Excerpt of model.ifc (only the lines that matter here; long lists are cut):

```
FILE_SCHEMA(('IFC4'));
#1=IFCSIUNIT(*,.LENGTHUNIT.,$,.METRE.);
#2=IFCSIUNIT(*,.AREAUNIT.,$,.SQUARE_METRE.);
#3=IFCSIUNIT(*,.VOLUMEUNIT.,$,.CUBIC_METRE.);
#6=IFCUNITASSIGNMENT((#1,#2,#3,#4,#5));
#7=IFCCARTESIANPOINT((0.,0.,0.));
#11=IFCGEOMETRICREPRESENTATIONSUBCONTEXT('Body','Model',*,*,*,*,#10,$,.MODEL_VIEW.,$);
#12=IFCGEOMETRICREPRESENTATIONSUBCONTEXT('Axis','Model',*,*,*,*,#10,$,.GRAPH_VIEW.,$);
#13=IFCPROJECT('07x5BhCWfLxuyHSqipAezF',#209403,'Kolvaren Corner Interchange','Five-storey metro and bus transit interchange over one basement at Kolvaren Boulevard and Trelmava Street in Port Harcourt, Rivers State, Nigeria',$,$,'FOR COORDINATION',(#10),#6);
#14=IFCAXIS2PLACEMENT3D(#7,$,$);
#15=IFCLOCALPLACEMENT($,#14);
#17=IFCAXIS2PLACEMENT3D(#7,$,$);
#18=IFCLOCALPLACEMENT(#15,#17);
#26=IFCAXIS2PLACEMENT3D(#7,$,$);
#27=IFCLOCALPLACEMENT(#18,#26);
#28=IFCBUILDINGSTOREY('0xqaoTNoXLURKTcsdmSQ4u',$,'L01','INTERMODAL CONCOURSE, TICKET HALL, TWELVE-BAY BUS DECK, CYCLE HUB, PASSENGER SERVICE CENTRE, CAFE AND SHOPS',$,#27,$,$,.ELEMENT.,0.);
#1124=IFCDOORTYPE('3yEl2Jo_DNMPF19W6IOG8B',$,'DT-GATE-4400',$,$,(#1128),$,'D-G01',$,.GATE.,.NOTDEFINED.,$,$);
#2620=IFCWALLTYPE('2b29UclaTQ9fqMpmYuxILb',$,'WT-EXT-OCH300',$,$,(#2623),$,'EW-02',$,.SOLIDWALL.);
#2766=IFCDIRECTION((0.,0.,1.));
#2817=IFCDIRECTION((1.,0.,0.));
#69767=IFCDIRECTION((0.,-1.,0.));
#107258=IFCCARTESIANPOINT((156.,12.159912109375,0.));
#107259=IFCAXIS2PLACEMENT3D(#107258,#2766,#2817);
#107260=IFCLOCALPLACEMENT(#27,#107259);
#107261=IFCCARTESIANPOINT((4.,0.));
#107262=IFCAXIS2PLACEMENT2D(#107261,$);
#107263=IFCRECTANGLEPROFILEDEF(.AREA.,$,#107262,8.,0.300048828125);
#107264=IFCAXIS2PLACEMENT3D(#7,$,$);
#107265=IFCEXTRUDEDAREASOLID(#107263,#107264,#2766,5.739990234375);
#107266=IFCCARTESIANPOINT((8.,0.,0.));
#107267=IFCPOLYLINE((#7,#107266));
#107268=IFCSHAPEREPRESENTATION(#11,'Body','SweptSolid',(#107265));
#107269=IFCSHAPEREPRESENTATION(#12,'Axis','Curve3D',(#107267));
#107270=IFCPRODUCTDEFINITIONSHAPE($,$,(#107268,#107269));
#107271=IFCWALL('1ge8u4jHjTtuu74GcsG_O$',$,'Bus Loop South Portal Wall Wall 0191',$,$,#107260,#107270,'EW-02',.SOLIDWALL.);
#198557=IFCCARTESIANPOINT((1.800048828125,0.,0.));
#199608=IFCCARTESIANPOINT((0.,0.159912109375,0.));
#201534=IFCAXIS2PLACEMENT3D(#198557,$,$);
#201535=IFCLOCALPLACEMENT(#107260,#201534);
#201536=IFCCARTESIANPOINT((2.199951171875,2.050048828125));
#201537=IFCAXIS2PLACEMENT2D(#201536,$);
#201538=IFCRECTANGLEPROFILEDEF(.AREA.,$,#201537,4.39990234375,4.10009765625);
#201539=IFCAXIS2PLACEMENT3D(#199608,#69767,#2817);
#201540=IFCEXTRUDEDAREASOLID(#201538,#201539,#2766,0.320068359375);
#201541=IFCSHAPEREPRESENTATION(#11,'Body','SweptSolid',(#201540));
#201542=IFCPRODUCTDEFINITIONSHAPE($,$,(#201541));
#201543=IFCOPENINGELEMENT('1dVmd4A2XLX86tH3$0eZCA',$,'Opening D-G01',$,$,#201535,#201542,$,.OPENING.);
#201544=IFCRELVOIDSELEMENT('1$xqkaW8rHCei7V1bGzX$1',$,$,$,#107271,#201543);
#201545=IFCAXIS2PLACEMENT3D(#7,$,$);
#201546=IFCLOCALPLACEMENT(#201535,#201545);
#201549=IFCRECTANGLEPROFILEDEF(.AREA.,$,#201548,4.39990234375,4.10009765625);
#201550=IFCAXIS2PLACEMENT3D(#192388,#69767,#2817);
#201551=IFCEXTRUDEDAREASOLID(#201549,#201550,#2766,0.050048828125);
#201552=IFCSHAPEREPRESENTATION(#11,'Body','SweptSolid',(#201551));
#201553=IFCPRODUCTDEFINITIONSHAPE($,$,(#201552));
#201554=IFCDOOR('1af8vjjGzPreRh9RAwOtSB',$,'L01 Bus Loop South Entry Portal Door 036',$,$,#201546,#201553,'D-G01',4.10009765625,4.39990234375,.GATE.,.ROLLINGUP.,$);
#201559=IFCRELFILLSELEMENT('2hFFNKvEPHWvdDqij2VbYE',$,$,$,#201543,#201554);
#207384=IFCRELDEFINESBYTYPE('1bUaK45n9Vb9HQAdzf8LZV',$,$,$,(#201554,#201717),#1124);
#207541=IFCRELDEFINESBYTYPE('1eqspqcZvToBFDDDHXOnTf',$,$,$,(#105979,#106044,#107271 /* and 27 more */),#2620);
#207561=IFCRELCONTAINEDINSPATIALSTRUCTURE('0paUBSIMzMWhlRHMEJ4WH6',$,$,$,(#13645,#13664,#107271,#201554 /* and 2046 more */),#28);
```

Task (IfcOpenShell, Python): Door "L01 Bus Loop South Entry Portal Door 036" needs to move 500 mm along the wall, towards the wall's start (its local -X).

```python
import ifcopenshell
import ifcopenshell.api.geometry
import ifcopenshell.util.placement

model = ifcopenshell.open("model.ifc")

door = model.by_id(201554)
opening = door.FillsVoids[0].RelatingOpeningElement
wall = opening.VoidsElements[0].RelatingBuildingElement

wall_matrix = ifcopenshell.util.placement.get_local_placement(wall.ObjectPlacement)
shift = wall_matrix[:3, 0] * -0.5
before = ifcopenshell.util.placement.get_local_placement(door.ObjectPlacement)[:3, 3].copy()

# The door is placed relative to its opening, so it follows when the opening moves.
matrix = ifcopenshell.util.placement.get_local_placement(opening.ObjectPlacement)
matrix[:3, 3] += shift
ifcopenshell.api.geometry.edit_object_placement(
    model, product=opening, matrix=matrix, is_si=False, should_transform_children=True
)

after = ifcopenshell.util.placement.get_local_placement(door.ObjectPlacement)[:3, 3]
print("door moved by", (after - before).round(3) + 0.0)

model.write("model-out.ifc")
```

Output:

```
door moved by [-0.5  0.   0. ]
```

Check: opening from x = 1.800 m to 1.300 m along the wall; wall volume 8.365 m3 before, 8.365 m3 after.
